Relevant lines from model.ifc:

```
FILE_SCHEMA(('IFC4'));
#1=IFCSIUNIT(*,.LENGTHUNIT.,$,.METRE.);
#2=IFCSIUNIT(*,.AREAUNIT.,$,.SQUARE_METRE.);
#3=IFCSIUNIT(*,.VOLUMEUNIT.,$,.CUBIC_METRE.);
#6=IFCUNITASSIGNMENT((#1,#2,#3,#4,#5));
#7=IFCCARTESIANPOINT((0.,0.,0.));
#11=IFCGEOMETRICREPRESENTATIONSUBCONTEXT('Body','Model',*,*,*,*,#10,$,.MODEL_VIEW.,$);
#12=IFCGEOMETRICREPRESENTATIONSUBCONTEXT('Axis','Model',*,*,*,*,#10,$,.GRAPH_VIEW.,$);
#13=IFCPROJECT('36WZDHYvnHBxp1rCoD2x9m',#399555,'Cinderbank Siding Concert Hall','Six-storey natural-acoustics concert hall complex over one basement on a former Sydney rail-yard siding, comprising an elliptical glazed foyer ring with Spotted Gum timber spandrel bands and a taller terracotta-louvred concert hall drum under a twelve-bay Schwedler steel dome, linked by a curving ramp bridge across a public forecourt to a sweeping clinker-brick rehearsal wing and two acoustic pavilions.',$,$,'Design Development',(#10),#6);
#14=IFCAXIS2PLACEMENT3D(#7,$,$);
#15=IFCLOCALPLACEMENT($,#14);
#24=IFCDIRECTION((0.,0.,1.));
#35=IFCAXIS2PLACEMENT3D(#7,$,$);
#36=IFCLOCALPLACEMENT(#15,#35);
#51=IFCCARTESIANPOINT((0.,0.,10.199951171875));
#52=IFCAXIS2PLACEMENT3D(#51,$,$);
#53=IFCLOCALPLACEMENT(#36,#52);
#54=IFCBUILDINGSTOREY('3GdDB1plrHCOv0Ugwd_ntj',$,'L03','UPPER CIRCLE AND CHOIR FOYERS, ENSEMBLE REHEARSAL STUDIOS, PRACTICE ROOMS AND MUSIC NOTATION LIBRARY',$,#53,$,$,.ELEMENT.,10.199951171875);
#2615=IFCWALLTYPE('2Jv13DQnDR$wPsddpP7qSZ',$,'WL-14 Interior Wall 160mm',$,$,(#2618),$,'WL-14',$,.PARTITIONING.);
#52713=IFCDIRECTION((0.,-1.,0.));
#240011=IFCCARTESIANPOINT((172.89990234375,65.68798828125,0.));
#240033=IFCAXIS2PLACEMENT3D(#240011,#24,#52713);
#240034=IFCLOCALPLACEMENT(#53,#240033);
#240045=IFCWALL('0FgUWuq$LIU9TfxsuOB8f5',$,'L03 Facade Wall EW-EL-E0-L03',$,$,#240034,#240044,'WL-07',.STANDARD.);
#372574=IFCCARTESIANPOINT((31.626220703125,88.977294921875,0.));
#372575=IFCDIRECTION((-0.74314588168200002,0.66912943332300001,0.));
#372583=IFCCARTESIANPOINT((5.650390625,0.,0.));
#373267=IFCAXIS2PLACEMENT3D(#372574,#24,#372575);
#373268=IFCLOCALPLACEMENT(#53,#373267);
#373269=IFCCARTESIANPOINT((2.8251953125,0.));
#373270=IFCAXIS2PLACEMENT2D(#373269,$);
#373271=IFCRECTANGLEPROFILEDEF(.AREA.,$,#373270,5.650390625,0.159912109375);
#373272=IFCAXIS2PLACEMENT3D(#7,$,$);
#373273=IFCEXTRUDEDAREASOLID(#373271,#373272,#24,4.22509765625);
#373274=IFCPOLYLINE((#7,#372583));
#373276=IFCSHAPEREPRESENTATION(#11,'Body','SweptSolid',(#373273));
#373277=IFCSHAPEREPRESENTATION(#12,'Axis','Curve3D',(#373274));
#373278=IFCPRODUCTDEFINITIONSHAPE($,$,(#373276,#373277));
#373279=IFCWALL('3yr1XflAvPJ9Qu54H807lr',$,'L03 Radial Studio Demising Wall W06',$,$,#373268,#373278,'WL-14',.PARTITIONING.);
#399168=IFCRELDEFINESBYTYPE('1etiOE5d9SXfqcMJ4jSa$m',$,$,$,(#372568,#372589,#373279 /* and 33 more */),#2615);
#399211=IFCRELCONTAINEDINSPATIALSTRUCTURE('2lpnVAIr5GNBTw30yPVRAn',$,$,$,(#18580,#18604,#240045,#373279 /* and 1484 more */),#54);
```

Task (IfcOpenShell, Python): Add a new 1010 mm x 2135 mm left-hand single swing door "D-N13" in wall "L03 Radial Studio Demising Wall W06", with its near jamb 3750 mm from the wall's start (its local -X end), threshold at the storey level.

```python
import numpy as np
import ifcopenshell
import ifcopenshell.api.feature
import ifcopenshell.api.geometry
import ifcopenshell.api.root
import ifcopenshell.api.spatial
import ifcopenshell.geom
import ifcopenshell.util.element
import ifcopenshell.util.placement
import ifcopenshell.util.representation
import ifcopenshell.util.shape
import ifcopenshell.util.unit

model = ifcopenshell.open("model.ifc")
unit_scale = ifcopenshell.util.unit.calculate_unit_scale(model)
settings = ifcopenshell.geom.settings()


def volume(element):
    """Net volume in cubic metres, openings subtracted."""
    shape = ifcopenshell.geom.create_shape(settings, element)
    return ifcopenshell.util.shape.get_volume(shape.geometry)


wall = model.by_guid("3yr1XflAvPJ9Qu54H807lr")
storey = ifcopenshell.util.element.get_container(wall, ifc_class="IfcBuildingStorey")
context = ifcopenshell.util.representation.get_context(model, "Model", "Body", "MODEL_VIEW")
before = volume(wall)

width, height, from_end, sill = 1.01, 2.135, 3.75, 0.0  # metres

# The wall runs along its own X axis, and the end named is its -X end.
wall_shape = ifcopenshell.geom.create_shape(settings, wall)
x, y, z = ifcopenshell.util.shape.get_vertices(wall_shape.geometry).T
start = x.min() + from_end
face, thickness = float(y.min()), float(y.max() - y.min())
wall_matrix = ifcopenshell.util.placement.get_local_placement(wall.ObjectPlacement)
level = ifcopenshell.util.placement.get_local_placement(storey.ObjectPlacement)[2, 3]


def in_wall(x, y):
    """Placement at x, y metres in the wall's axes, at sill height."""
    matrix = wall_matrix.copy()
    matrix[:, 3] = wall_matrix @ np.array([x / unit_scale, y / unit_scale, 0.0, 1.0])
    matrix[2, 3] = level + sill / unit_scale
    return matrix


# Opening: a box that overshoots both wall faces by 50 mm.
opening = ifcopenshell.api.root.create_entity(model, ifc_class="IfcOpeningElement", predefined_type="OPENING")
box = ifcopenshell.api.geometry.add_wall_representation(
    model, context=context, length=width, height=height, thickness=thickness + 0.1
)
ifcopenshell.api.geometry.assign_representation(model, product=opening, representation=box)
ifcopenshell.api.geometry.edit_object_placement(model, product=opening, matrix=in_wall(start, face - 0.05), is_si=False)
ifcopenshell.api.feature.add_feature(model, feature=opening, element=wall)

door = ifcopenshell.api.root.create_entity(model, ifc_class="IfcDoor", name="D-N13", predefined_type="DOOR")
door.OverallWidth, door.OverallHeight = width / unit_scale, height / unit_scale
door.OperationType = "SINGLE_SWING_LEFT"
body = ifcopenshell.api.geometry.add_door_representation(
    model,
    context=context,
    overall_width=door.OverallWidth,
    overall_height=door.OverallHeight,
    operation_type="SINGLE_SWING_LEFT",
    lining_properties={"LiningDepth": thickness / unit_scale, "ThresholdDepth": thickness / unit_scale},
)
ifcopenshell.api.geometry.assign_representation(model, product=door, representation=body)
ifcopenshell.api.spatial.assign_container(model, products=[door], relating_structure=storey)
ifcopenshell.api.feature.add_filling(model, opening=opening, element=door)

# The lining spans the wall, so the door starts at the wall face.
ifcopenshell.api.geometry.edit_object_placement(model, product=door, matrix=in_wall(start, face), is_si=False)

after = volume(wall)

print(f"wall volume {before:.3f} -> {after:.3f} m3")

model.write("model_edited.ifc")
```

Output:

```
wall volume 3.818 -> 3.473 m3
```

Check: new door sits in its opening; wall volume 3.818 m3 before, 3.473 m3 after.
